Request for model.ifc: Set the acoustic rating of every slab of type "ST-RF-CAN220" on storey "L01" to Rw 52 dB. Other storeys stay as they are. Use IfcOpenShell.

First a look at what the model holds.

```python
import ifcopenshell
import ifcopenshell.util.element

model = ifcopenshell.open("model.ifc")
print(model.schema)
storey = next(s for s in model.by_type("IfcBuildingStorey") if s.Name == "L01")
slabs = [e for e in ifcopenshell.util.element.get_decomposition(storey) if e.is_a("IfcSlab")]
seen = {}
for e in slabs:
    element_type = ifcopenshell.util.element.get_type(e)
    key = (element_type.Name if element_type != e and element_type else None, ifcopenshell.util.element.get_pset(e, "Pset_SlabCommon", "AcousticRating"))
    seen[key] = seen.get(key, 0) + 1
for (name, value), count in sorted(seen.items(), key=str):
    print(count, "x", name, "|", value)
```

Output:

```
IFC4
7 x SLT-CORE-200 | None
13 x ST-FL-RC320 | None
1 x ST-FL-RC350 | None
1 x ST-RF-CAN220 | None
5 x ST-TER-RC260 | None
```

```python
import ifcopenshell
import ifcopenshell.api.pset
import ifcopenshell.util.element

model = ifcopenshell.open("model.ifc")

storey = next(s for s in model.by_type("IfcBuildingStorey") if s.Name == "L01")
slabs = [e for e in ifcopenshell.util.element.get_decomposition(storey) if e.is_a("IfcSlab")]

count = 0
for e in slabs:
    element_type = ifcopenshell.util.element.get_type(e)
    if element_type in (None, e) or element_type.Name != "ST-RF-CAN220":
        continue
    # add_pset returns the element's existing set when there is one.
    pset = ifcopenshell.api.pset.add_pset(model, product=e, name="Pset_SlabCommon")
    ifcopenshell.api.pset.edit_pset(model, pset=pset, properties={"AcousticRating": "Rw 52 dB"})
    count += 1

print(count, "slabs updated")

model.write("model_rev.ifc")
```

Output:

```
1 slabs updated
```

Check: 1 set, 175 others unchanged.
